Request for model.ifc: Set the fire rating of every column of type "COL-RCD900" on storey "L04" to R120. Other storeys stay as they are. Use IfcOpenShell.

First a look at what the model holds.

```python
import ifcopenshell
import ifcopenshell.util.element

model = ifcopenshell.open("model.ifc")
print(model.schema)
storey = next(s for s in model.by_type("IfcBuildingStorey") if s.Name == "L04")
columns = [e for e in ifcopenshell.util.element.get_decomposition(storey) if e.is_a("IfcColumn")]
seen = {}
for e in columns:
    element_type = ifcopenshell.util.element.get_type(e)
    key = (element_type.Name if element_type != e and element_type else None, ifcopenshell.util.element.get_pset(e, "Pset_ColumnCommon", "FireRating"))
    seen[key] = seen.get(key, 0) + 1
for (name, value), count in sorted(seen.items(), key=str):
    print(count, "x", name, "|", value)
```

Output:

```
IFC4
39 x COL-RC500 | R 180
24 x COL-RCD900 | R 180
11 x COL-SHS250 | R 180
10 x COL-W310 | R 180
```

```python
import ifcopenshell
import ifcopenshell.api.pset
import ifcopenshell.util.element

model = ifcopenshell.open("model.ifc")

storey = next(s for s in model.by_type("IfcBuildingStorey") if s.Name == "L04")
columns = [e for e in ifcopenshell.util.element.get_decomposition(storey) if e.is_a("IfcColumn")]

count = 0
for e in columns:
    element_type = ifcopenshell.util.element.get_type(e)
    if element_type in (None, e) or element_type.Name != "COL-RCD900":
        continue
    # add_pset returns the element's existing set when there is one.
    pset = ifcopenshell.api.pset.add_pset(model, product=e, name="Pset_ColumnCommon")
    ifcopenshell.api.pset.edit_pset(model, pset=pset, properties={"FireRating": "R120"})
    count += 1

print(count, "columns updated")

model.write("model_rev.ifc")
```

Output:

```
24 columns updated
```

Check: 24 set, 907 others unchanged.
